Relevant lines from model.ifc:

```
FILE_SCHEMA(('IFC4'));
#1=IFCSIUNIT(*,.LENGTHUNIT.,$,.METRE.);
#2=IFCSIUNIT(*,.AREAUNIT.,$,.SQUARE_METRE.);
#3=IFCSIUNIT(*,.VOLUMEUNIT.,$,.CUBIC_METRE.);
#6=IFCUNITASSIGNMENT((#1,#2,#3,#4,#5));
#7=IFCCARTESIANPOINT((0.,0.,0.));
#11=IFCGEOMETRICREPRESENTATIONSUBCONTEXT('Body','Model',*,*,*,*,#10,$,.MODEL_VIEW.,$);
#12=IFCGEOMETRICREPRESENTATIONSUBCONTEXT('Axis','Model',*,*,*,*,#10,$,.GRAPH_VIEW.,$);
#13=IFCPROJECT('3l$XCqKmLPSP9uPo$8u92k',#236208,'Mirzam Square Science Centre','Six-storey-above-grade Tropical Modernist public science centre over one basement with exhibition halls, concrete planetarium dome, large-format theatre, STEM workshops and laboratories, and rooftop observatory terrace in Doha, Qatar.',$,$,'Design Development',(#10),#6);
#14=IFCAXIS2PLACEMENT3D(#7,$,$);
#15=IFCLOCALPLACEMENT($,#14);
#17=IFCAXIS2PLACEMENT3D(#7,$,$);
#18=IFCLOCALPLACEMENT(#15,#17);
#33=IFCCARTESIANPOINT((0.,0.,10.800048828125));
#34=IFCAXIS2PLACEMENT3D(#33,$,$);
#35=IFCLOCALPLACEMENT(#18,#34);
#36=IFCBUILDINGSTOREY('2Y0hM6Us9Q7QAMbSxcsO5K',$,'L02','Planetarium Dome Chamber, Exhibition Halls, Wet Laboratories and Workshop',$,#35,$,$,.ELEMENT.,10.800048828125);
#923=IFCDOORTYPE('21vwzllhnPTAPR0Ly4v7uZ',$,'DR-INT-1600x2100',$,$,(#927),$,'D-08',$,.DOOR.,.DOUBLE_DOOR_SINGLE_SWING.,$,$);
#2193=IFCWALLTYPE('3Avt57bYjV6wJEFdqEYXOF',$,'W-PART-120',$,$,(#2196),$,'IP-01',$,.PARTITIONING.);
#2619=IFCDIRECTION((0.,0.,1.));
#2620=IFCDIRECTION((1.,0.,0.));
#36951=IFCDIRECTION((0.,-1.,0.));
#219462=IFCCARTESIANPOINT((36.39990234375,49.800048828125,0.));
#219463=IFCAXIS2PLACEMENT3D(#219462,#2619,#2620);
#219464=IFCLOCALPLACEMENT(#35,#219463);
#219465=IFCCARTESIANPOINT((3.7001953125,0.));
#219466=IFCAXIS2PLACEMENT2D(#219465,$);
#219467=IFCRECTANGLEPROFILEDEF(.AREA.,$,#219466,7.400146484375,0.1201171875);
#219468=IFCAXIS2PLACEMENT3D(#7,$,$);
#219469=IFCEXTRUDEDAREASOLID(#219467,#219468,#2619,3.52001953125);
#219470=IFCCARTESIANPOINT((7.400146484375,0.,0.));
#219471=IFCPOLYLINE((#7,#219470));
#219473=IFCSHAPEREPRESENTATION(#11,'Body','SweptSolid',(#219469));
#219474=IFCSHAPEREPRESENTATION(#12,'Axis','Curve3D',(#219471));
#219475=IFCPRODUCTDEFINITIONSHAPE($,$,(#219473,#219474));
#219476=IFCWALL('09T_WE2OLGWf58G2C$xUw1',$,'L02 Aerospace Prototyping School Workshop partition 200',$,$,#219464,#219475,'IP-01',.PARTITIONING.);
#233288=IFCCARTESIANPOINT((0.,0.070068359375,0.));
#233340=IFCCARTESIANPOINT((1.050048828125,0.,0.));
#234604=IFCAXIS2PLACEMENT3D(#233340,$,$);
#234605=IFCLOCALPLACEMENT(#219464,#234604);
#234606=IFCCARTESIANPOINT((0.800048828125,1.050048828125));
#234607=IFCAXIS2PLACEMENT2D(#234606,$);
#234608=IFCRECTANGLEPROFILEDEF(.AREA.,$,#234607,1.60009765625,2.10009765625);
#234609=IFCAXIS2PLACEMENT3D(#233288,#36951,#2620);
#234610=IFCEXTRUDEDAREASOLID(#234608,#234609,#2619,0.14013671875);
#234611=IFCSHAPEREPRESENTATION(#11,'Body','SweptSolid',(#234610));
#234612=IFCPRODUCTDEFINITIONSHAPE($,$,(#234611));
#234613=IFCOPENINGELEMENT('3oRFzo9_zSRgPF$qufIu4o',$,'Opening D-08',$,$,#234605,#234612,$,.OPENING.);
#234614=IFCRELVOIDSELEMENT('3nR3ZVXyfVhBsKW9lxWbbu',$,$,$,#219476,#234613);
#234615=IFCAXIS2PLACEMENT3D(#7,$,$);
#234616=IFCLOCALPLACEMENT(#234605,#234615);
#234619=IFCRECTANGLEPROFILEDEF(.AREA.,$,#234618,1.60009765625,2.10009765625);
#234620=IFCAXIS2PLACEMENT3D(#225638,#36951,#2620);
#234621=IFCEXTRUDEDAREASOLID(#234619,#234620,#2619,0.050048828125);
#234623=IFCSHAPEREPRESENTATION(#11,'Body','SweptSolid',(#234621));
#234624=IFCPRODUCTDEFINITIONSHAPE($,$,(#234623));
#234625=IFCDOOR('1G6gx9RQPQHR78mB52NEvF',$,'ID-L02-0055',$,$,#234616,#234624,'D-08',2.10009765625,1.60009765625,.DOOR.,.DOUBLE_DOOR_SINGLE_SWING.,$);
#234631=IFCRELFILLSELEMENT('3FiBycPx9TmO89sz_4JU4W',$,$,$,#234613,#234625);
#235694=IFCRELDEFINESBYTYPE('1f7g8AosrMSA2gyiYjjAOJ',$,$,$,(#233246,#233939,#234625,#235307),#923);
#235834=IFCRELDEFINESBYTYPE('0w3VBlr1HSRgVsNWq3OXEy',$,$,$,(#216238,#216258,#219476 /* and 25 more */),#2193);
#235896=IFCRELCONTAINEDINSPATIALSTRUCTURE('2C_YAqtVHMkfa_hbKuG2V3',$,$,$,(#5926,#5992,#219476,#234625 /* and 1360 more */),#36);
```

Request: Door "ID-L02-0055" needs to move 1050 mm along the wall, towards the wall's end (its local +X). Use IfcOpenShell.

```python
import ifcopenshell
import ifcopenshell.api.geometry
import ifcopenshell.util.placement
import ifcopenshell.util.unit

model = ifcopenshell.open("model.ifc")
unit_scale = ifcopenshell.util.unit.calculate_unit_scale(model)

door = model.by_guid("1G6gx9RQPQHR78mB52NEvF")
opening = door.FillsVoids[0].RelatingOpeningElement
wall = opening.VoidsElements[0].RelatingBuildingElement

wall_matrix = ifcopenshell.util.placement.get_local_placement(wall.ObjectPlacement)
shift = wall_matrix[:3, 0] * 1.05 / unit_scale
before = ifcopenshell.util.placement.get_local_placement(door.ObjectPlacement)[:3, 3].copy()

# The door is placed relative to its opening, so it follows when the opening moves.
matrix = ifcopenshell.util.placement.get_local_placement(opening.ObjectPlacement)
matrix[:3, 3] += shift
ifcopenshell.api.geometry.edit_object_placement(
    model, product=opening, matrix=matrix, is_si=False, should_transform_children=True
)

after = ifcopenshell.util.placement.get_local_placement(door.ObjectPlacement)[:3, 3]
print("door moved by", (after - before).round(3) + 0.0)

model.write("model_v2.ifc")
```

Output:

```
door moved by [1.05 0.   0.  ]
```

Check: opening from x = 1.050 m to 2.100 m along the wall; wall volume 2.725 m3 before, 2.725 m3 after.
